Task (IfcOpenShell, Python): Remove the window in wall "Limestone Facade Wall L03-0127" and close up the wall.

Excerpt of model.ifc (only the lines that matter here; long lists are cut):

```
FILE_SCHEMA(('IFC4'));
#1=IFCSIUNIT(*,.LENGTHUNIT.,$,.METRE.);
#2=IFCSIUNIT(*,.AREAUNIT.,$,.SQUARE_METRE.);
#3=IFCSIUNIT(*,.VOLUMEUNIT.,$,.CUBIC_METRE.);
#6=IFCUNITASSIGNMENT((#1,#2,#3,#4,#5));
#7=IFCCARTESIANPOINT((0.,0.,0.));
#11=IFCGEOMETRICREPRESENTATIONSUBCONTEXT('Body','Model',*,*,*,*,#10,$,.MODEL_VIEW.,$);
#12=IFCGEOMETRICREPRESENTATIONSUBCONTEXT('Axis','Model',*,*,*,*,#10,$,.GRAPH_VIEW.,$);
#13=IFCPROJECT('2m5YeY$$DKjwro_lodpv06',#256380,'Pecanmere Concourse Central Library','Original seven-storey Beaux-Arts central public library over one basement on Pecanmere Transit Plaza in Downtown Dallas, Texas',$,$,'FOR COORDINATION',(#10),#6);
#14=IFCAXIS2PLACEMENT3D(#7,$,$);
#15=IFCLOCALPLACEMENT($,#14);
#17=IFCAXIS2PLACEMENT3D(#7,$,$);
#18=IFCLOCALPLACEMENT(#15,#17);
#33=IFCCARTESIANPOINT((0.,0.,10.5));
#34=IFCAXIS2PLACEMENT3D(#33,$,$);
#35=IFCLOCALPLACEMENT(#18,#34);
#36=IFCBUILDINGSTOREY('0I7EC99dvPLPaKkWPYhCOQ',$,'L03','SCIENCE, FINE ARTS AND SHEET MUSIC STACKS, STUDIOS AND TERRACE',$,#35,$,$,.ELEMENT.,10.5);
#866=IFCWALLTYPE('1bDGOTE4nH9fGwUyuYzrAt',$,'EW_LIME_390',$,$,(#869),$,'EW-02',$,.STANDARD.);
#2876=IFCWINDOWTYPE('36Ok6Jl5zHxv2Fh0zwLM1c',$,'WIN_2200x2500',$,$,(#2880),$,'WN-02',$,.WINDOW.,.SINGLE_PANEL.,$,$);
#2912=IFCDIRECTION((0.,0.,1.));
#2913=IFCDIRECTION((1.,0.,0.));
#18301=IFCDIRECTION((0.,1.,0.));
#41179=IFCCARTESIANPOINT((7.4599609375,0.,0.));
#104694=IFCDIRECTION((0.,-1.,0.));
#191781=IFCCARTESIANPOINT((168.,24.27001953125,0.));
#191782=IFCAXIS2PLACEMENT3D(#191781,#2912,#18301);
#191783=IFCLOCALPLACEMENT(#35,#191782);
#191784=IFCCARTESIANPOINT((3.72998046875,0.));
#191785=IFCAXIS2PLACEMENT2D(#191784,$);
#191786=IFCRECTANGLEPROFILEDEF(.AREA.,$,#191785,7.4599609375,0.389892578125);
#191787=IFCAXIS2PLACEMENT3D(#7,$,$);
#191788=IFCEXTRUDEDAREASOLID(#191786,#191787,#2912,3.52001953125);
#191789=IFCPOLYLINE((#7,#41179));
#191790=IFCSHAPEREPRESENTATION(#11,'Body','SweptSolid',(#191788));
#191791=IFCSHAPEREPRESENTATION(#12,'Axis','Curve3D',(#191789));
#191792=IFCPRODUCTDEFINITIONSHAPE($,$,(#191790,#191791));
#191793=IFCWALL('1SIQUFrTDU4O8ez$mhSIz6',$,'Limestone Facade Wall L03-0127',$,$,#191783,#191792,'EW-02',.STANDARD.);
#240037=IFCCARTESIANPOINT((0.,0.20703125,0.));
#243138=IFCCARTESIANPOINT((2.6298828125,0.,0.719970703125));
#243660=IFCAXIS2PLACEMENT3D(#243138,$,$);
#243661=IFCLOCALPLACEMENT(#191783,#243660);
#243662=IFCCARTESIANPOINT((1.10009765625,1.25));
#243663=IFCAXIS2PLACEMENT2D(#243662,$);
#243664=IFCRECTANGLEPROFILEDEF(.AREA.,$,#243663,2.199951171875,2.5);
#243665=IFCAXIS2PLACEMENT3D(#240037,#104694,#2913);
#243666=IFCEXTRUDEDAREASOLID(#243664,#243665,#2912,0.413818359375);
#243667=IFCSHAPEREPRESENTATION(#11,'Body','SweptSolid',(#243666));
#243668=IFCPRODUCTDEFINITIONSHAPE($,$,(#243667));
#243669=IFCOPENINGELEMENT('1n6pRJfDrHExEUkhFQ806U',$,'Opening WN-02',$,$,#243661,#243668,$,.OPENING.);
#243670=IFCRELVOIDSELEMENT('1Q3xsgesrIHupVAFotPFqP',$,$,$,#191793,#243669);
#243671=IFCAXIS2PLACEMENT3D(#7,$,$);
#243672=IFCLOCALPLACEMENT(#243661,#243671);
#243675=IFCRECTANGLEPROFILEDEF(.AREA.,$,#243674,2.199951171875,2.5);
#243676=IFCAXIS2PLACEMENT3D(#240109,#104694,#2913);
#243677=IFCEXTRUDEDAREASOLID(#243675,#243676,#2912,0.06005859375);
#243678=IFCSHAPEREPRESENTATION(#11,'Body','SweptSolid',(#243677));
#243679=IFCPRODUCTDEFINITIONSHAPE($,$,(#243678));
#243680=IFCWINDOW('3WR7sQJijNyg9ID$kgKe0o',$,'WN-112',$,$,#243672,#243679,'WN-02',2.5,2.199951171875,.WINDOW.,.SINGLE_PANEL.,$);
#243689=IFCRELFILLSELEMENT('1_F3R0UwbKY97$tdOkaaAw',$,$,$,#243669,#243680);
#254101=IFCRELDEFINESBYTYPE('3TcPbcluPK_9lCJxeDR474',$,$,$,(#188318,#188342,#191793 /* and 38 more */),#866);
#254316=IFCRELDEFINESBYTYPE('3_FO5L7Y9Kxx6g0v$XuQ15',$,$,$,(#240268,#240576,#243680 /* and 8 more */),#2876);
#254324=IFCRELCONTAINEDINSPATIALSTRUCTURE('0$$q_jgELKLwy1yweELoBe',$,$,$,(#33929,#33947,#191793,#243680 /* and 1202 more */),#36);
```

```python
import ifcopenshell
import ifcopenshell.api.feature
import ifcopenshell.api.root
import ifcopenshell.geom
import ifcopenshell.util.shape

model = ifcopenshell.open("model.ifc")
settings = ifcopenshell.geom.settings()


def volume(element):
    """Net volume in cubic metres, openings subtracted."""
    shape = ifcopenshell.geom.create_shape(settings, element)
    return ifcopenshell.util.shape.get_volume(shape.geometry)


window = model.by_id(243680)
opening = window.FillsVoids[0].RelatingOpeningElement
wall = opening.VoidsElements[0].RelatingBuildingElement
before = volume(wall)

ifcopenshell.api.root.remove_product(model, product=window)
ifcopenshell.api.feature.remove_feature(model, feature=opening)

after = volume(wall)

print(f"wall volume {before:.3f} -> {after:.3f} m3")

model.write("model_edited.ifc")
```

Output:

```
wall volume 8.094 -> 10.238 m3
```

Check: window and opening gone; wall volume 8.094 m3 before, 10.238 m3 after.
